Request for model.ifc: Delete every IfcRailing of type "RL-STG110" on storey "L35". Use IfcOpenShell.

First a look at what the model holds.

```python
import ifcopenshell
import ifcopenshell.util.element

model = ifcopenshell.open("model.ifc")
print(model.schema)
storey = next(s for s in model.by_type("IfcBuildingStorey") if s.Name == "L35")
railings = [e for e in ifcopenshell.util.element.get_decomposition(storey) if e.is_a("IfcRailing")]
seen = {}
for e in railings:
    element_type = ifcopenshell.util.element.get_type(e)
    name = element_type.Name if element_type not in (None, e) else None
    seen[name] = seen.get(name, 0) + 1
for name, count in sorted(seen.items(), key=str):
    print(count, "x", name)
```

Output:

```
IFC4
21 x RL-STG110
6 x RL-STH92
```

```python
import ifcopenshell
import ifcopenshell.api.root
import ifcopenshell.util.element

model = ifcopenshell.open("model.ifc")

storey = next(s for s in model.by_type("IfcBuildingStorey") if s.Name == "L35")
railings = [e for e in ifcopenshell.util.element.get_decomposition(storey) if e.is_a("IfcRailing")]
targets = [e for e in railings if (t := ifcopenshell.util.element.get_type(e)) not in (None, e) and t.Name == "RL-STG110"]

for e in targets:
    ifcopenshell.api.root.remove_product(model, product=e)
print(len(targets), "removed")

model.write("model_rev.ifc")
```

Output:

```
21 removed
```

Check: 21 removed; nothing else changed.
